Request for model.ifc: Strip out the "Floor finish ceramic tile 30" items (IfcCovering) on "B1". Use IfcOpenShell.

First a look at what the model holds.

```python
import ifcopenshell
import ifcopenshell.util.element

model = ifcopenshell.open("model.ifc")
print(model.schema)
storey = next(s for s in model.by_type("IfcBuildingStorey") if s.Name == "B1")
coverings = [e for e in ifcopenshell.util.element.get_decomposition(storey) if e.is_a("IfcCovering")]
seen = {}
for e in coverings:
    element_type = ifcopenshell.util.element.get_type(e)
    name = element_type.Name if element_type not in (None, e) else None
    seen[name] = seen.get(name, 0) + 1
for name, count in sorted(seen.items(), key=str):
    print(count, "x", name)
```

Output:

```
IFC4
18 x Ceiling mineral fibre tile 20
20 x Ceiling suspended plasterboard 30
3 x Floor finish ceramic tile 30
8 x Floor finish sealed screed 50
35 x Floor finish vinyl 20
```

```python
import ifcopenshell
import ifcopenshell.api.root
import ifcopenshell.util.element

model = ifcopenshell.open("model.ifc")

storey = next(s for s in model.by_type("IfcBuildingStorey") if s.Name == "B1")
coverings = [e for e in ifcopenshell.util.element.get_decomposition(storey) if e.is_a("IfcCovering")]
targets = [e for e in coverings if (t := ifcopenshell.util.element.get_type(e)) not in (None, e) and t.Name == "Floor finish ceramic tile 30"]

for e in targets:
    ifcopenshell.api.root.remove_product(model, product=e)
print(len(targets), "removed")

model.write("model_edited.ifc")
```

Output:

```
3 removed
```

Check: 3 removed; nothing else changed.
